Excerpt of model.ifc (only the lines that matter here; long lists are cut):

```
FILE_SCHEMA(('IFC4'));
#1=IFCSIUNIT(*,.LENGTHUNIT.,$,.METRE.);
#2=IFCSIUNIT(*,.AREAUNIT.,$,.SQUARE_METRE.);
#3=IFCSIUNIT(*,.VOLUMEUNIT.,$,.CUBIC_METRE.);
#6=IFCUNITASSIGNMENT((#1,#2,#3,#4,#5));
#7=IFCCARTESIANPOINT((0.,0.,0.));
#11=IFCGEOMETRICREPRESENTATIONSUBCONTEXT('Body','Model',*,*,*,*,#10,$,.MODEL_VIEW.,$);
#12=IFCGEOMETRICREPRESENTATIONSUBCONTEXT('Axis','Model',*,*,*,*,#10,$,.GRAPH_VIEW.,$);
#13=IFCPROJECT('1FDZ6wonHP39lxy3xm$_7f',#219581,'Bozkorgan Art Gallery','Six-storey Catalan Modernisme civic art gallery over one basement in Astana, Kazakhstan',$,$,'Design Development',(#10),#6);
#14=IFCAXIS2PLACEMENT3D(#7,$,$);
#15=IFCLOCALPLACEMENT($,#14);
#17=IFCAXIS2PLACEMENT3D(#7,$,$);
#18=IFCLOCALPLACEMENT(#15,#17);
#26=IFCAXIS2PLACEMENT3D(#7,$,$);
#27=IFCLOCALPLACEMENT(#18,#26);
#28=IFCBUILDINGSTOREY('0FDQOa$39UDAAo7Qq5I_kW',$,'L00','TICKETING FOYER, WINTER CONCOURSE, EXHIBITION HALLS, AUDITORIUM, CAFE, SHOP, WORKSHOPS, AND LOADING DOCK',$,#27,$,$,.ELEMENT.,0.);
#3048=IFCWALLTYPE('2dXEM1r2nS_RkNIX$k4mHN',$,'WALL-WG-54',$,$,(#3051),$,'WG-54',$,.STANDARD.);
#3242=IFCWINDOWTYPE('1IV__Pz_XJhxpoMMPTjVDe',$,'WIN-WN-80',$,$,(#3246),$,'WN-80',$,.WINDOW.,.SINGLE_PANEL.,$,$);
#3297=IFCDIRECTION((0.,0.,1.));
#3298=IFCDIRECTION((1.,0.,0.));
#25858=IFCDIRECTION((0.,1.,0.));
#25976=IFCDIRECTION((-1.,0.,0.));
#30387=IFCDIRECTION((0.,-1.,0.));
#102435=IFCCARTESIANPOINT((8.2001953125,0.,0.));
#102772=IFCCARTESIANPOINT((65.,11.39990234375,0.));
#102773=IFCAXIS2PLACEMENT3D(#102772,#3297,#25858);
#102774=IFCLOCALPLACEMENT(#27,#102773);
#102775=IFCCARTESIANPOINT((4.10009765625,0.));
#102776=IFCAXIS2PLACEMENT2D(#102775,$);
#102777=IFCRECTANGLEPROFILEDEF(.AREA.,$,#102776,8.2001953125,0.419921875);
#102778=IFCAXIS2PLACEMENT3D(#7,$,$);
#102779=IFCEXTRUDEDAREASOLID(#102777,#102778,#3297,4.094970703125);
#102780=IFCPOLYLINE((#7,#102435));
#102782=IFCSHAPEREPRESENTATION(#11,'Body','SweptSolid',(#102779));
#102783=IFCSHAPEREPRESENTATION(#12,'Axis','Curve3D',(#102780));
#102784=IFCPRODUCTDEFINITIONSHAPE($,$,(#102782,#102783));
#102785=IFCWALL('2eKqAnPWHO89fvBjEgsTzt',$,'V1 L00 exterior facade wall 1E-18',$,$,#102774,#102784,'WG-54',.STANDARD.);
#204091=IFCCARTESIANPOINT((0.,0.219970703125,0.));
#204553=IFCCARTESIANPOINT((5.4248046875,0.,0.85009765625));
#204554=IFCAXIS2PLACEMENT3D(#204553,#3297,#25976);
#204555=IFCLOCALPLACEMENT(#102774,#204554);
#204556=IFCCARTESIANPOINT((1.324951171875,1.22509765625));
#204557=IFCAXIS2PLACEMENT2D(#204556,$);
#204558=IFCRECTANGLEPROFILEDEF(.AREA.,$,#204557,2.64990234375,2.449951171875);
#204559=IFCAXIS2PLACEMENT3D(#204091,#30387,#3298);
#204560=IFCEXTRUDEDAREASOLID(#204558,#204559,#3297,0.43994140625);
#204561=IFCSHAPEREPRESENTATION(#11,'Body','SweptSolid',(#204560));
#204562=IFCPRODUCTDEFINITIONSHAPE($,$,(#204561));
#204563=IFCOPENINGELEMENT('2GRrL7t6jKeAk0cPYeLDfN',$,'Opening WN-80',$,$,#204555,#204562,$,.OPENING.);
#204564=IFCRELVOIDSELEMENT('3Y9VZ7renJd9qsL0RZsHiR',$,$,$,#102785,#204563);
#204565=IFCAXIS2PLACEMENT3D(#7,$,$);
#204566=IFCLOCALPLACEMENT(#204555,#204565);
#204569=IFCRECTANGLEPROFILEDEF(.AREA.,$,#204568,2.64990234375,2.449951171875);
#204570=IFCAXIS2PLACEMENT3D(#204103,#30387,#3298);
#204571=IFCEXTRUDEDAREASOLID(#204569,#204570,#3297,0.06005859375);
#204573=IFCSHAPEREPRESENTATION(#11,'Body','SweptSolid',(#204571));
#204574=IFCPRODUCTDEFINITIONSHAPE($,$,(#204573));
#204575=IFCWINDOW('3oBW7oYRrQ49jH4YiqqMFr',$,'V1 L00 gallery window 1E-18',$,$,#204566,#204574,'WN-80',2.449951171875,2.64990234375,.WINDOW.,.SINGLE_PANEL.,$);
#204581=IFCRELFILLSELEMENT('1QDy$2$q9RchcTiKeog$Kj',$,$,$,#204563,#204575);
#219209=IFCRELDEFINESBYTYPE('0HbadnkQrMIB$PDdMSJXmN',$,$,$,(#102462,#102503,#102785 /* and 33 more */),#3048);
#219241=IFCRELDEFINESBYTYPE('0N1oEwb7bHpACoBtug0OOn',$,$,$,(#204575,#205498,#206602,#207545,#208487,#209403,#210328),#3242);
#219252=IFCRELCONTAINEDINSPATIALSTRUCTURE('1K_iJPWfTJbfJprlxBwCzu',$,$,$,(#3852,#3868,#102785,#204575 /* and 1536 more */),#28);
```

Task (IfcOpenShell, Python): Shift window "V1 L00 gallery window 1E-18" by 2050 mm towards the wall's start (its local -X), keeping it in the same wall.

```python
import ifcopenshell
import ifcopenshell.api.geometry
import ifcopenshell.util.placement

model = ifcopenshell.open("model.ifc")

window = model.by_guid("3oBW7oYRrQ49jH4YiqqMFr")
opening = window.FillsVoids[0].RelatingOpeningElement
wall = opening.VoidsElements[0].RelatingBuildingElement

wall_matrix = ifcopenshell.util.placement.get_local_placement(wall.ObjectPlacement)
shift = wall_matrix[:3, 0] * -2.05
before = ifcopenshell.util.placement.get_local_placement(window.ObjectPlacement)[:3, 3].copy()

# The window is placed relative to its opening, so it follows when the opening moves.
matrix = ifcopenshell.util.placement.get_local_placement(opening.ObjectPlacement)
matrix[:3, 3] += shift
ifcopenshell.api.geometry.edit_object_placement(
    model, product=opening, matrix=matrix, is_si=False, should_transform_children=True
)

after = ifcopenshell.util.placement.get_local_placement(window.ObjectPlacement)[:3, 3]
print("window moved by", (after - before).round(3) + 0.0)

model.write("model_updated.ifc")
```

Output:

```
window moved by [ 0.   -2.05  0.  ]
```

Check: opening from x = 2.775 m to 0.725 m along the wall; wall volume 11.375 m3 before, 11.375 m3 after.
